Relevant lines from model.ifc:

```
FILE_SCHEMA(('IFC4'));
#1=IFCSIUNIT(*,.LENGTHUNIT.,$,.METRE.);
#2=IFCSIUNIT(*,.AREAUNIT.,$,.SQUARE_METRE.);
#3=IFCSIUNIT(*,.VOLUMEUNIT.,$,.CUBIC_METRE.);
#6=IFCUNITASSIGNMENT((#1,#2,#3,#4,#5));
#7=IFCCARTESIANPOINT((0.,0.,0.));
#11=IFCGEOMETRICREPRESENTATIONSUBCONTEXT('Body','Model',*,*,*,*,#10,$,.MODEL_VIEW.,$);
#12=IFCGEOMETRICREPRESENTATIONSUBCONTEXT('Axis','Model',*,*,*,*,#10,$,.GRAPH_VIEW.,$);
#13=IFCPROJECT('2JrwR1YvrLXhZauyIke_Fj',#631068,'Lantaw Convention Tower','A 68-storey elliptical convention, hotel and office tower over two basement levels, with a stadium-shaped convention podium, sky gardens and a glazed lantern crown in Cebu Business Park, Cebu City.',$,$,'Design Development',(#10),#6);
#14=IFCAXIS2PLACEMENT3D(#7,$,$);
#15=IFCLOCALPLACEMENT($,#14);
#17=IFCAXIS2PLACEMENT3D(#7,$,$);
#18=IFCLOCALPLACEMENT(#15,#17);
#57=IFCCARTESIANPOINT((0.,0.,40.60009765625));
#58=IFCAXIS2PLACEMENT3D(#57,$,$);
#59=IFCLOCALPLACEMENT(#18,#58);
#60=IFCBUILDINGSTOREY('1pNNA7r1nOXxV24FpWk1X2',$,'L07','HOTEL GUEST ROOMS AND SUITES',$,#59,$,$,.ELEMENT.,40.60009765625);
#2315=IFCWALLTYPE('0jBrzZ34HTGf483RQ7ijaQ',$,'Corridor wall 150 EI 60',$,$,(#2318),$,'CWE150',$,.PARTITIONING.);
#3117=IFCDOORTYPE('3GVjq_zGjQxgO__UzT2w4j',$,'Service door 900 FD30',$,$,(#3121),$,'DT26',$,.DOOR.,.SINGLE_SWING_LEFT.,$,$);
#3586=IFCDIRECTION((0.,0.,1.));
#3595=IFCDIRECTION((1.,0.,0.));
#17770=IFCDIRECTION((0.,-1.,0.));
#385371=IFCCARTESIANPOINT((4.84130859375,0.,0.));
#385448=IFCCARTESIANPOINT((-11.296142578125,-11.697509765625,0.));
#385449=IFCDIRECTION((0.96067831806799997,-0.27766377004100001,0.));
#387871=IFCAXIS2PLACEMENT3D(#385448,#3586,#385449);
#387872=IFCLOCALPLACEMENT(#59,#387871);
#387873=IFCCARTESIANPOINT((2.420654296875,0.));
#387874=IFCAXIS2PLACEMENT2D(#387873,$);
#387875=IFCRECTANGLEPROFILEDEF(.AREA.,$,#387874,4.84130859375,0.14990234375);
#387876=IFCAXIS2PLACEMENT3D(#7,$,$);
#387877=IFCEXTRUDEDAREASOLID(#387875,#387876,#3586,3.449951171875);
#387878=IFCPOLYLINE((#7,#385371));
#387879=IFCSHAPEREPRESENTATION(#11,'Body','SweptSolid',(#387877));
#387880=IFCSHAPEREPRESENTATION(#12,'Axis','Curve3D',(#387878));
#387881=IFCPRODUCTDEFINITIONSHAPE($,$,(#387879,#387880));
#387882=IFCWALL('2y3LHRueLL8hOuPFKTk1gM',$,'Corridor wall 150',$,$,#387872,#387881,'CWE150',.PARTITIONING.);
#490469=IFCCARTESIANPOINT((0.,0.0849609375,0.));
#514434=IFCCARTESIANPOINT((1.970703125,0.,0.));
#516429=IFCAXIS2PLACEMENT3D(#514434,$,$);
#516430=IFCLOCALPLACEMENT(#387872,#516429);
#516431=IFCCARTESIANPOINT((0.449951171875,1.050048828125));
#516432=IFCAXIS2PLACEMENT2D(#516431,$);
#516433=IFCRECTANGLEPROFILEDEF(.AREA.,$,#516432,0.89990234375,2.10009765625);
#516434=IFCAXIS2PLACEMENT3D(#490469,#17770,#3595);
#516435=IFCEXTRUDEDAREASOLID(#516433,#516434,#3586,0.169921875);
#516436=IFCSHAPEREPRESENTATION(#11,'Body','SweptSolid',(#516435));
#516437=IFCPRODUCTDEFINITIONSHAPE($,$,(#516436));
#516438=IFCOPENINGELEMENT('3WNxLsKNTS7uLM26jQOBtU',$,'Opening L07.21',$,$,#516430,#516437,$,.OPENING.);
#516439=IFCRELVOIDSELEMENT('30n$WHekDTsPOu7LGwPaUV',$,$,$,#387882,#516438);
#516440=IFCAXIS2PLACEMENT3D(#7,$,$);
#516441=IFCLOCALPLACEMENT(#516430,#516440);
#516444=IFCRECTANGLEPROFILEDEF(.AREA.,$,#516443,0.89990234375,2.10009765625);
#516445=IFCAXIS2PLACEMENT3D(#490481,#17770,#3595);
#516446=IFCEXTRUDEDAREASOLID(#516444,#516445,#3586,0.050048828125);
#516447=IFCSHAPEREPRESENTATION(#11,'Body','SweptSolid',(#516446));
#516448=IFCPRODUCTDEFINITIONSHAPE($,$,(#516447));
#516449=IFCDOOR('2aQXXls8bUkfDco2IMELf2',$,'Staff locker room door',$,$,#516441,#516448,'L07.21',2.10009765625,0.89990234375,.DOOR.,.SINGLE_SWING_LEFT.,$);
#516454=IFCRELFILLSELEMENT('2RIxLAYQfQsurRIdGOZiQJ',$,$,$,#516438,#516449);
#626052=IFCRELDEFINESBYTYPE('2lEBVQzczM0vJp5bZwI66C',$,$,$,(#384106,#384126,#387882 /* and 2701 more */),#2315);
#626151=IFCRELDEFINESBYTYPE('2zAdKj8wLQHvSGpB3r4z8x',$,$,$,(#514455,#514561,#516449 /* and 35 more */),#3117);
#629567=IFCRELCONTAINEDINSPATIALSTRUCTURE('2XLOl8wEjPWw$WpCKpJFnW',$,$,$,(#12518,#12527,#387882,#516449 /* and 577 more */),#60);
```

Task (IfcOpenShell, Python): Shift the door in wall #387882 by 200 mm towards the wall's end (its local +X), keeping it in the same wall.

```python
import ifcopenshell
import ifcopenshell.api.geometry
import ifcopenshell.util.placement

model = ifcopenshell.open("model.ifc")

door = model.by_guid("2aQXXls8bUkfDco2IMELf2")
opening = door.FillsVoids[0].RelatingOpeningElement
wall = opening.VoidsElements[0].RelatingBuildingElement

wall_matrix = ifcopenshell.util.placement.get_local_placement(wall.ObjectPlacement)
shift = wall_matrix[:3, 0] * 0.2
before = ifcopenshell.util.placement.get_local_placement(door.ObjectPlacement)[:3, 3].copy()

# The door is placed relative to its opening, so it follows when the opening moves.
matrix = ifcopenshell.util.placement.get_local_placement(opening.ObjectPlacement)
matrix[:3, 3] += shift
ifcopenshell.api.geometry.edit_object_placement(
    model, product=opening, matrix=matrix, is_si=False, should_transform_children=True
)

after = ifcopenshell.util.placement.get_local_placement(door.ObjectPlacement)[:3, 3]
print("door moved by", (after - before).round(3) + 0.0)

model.write("model_rev.ifc")
```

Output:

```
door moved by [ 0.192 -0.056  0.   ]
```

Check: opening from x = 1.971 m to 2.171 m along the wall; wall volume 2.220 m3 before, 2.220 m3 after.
